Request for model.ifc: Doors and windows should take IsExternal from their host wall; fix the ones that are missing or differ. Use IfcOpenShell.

First a look at what the model holds.

```python
import ifcopenshell
import ifcopenshell.util.element

model = ifcopenshell.open("model.ifc")
print(model.schema)
seen = {}
for e in model.by_type("IfcDoor") + model.by_type("IfcWindow"):
    if not e.FillsVoids:
        continue
    host = e.FillsVoids[0].RelatingOpeningElement.VoidsElements[0].RelatingBuildingElement
    own = ifcopenshell.util.element.get_pset(e, f"Pset_{e.is_a()[3:].removesuffix('StandardCase')}Common", "IsExternal")
    wall = ifcopenshell.util.element.get_pset(host, "Pset_WallCommon", "IsExternal")
    seen[e.is_a(), own, wall] = seen.get((e.is_a(), own, wall), 0) + 1
for (cls, own, wall), count in sorted(seen.items(), key=str):
    print(count, cls, "IsExternal:", own, "| host wall:", wall)
```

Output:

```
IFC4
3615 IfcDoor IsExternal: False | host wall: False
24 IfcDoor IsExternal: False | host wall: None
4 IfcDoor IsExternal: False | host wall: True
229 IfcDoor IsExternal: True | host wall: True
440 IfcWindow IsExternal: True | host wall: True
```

```python
import ifcopenshell
import ifcopenshell.api.pset
import ifcopenshell.util.element

model = ifcopenshell.open("model.ifc")

count = 0
for ifc_class, pset_name in (("IfcDoor", "Pset_DoorCommon"), ("IfcWindow", "Pset_WindowCommon")):
    for e in model.by_type(ifc_class):
        if not e.FillsVoids:
            continue
        host = e.FillsVoids[0].RelatingOpeningElement.VoidsElements[0].RelatingBuildingElement
        external = ifcopenshell.util.element.get_pset(host, "Pset_WallCommon", "IsExternal")
        if external is None or ifcopenshell.util.element.get_pset(e, pset_name, "IsExternal") == external:
            continue
        pset = ifcopenshell.api.pset.add_pset(model, product=e, name=pset_name)
        ifcopenshell.api.pset.edit_pset(model, pset=pset, properties={"IsExternal": external})
        count += 1

print(count, "updated")

model.write("model_edited.ifc")
```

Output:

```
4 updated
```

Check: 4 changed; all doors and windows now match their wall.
